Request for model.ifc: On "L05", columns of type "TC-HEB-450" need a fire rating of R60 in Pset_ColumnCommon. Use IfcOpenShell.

First a look at what the model holds.

```python
import ifcopenshell
import ifcopenshell.util.element

model = ifcopenshell.open("model.ifc")
print(model.schema)
storey = next(s for s in model.by_type("IfcBuildingStorey") if s.Name == "L05")
columns = [e for e in ifcopenshell.util.element.get_decomposition(storey) if e.is_a("IfcColumn")]
seen = {}
for e in columns:
    element_type = ifcopenshell.util.element.get_type(e)
    key = (element_type.Name if element_type != e and element_type else None, ifcopenshell.util.element.get_pset(e, "Pset_ColumnCommon", "FireRating"))
    seen[key] = seen.get(key, 0) + 1
for (name, value), count in sorted(seen.items(), key=str):
    print(count, "x", name, "|", value)
```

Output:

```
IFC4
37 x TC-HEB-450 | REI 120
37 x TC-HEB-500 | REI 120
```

```python
import ifcopenshell
import ifcopenshell.api.pset
import ifcopenshell.util.element

model = ifcopenshell.open("model.ifc")

storey = next(s for s in model.by_type("IfcBuildingStorey") if s.Name == "L05")
columns = [e for e in ifcopenshell.util.element.get_decomposition(storey) if e.is_a("IfcColumn")]

count = 0
for e in columns:
    element_type = ifcopenshell.util.element.get_type(e)
    if element_type in (None, e) or element_type.Name != "TC-HEB-450":
        continue
    # add_pset returns the element's existing set when there is one.
    pset = ifcopenshell.api.pset.add_pset(model, product=e, name="Pset_ColumnCommon")
    ifcopenshell.api.pset.edit_pset(model, pset=pset, properties={"FireRating": "R60"})
    count += 1

print(count, "columns updated")

model.write("model_updated.ifc")
```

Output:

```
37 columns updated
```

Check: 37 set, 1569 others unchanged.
